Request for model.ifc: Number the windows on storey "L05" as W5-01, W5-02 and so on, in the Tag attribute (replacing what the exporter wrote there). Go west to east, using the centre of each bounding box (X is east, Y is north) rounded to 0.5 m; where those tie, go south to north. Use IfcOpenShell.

First a look at what the model holds.

```python
import ifcopenshell
import ifcopenshell.util.element
import ifcopenshell.util.placement

model = ifcopenshell.open("model.ifc")
print(model.schema)
storey = next(s for s in model.by_type("IfcBuildingStorey") if s.Name == "L05")
windows = [e for e in ifcopenshell.util.element.get_decomposition(storey) if e.is_a("IfcWindow")]
for e in sorted(windows, key=lambda e: e.id()):
    origin = ifcopenshell.util.placement.get_local_placement(e.ObjectPlacement)[:3, 3]
    print(e.id(), e.Tag, e.Name, origin.round(2) + 0.0, sep=" | ")
```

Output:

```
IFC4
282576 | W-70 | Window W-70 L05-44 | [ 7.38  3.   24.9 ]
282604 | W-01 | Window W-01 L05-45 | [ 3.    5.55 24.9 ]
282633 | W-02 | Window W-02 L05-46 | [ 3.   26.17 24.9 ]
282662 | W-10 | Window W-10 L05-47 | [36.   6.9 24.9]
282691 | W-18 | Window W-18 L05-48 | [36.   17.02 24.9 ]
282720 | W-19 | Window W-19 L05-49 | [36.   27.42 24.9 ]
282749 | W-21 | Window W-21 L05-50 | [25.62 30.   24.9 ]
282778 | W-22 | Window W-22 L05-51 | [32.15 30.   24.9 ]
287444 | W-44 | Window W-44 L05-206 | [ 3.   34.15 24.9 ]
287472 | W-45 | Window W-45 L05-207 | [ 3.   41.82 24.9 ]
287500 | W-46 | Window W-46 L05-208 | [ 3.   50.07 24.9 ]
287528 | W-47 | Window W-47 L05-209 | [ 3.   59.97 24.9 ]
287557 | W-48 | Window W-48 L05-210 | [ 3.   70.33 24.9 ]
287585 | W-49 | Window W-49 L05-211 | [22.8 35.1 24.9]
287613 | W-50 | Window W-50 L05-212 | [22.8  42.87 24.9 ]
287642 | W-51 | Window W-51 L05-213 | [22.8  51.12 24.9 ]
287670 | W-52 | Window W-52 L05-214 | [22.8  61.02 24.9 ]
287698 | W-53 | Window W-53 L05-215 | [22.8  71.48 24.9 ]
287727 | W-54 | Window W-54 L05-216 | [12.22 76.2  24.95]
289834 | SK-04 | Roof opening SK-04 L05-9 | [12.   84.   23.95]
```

```python
import ifcopenshell
import ifcopenshell.geom
import ifcopenshell.util.element
import ifcopenshell.util.shape

model = ifcopenshell.open("model.ifc")
settings = ifcopenshell.geom.settings()
settings.set("use-world-coords", True)


def centre(element):
    shape = ifcopenshell.geom.create_shape(settings, element)
    return ifcopenshell.util.shape.get_bbox_centroid(shape.geometry)


storey = next(s for s in model.by_type("IfcBuildingStorey") if s.Name == "L05")
windows = [e for e in ifcopenshell.util.element.get_decomposition(storey) if e.is_a("IfcWindow")]

# Insertion points can sit at a corner or the storey origin, so sort by the geometry (in metres).
centres = {e: centre(e) for e in windows}
windows.sort(key=lambda e: (round(centres[e][0] / 0.5), centres[e][1]))

for i, e in enumerate(windows, start=1):
    number = f"W5-{i:02d}"
    e.Tag = number
    print(e.id(), number)

model.write("model_edited.ifc")
```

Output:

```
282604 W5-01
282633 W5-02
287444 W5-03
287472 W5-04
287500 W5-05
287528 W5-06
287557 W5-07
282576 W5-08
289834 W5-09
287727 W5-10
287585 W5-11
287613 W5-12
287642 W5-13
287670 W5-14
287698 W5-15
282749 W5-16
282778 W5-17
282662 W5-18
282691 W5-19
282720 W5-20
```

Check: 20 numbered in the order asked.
